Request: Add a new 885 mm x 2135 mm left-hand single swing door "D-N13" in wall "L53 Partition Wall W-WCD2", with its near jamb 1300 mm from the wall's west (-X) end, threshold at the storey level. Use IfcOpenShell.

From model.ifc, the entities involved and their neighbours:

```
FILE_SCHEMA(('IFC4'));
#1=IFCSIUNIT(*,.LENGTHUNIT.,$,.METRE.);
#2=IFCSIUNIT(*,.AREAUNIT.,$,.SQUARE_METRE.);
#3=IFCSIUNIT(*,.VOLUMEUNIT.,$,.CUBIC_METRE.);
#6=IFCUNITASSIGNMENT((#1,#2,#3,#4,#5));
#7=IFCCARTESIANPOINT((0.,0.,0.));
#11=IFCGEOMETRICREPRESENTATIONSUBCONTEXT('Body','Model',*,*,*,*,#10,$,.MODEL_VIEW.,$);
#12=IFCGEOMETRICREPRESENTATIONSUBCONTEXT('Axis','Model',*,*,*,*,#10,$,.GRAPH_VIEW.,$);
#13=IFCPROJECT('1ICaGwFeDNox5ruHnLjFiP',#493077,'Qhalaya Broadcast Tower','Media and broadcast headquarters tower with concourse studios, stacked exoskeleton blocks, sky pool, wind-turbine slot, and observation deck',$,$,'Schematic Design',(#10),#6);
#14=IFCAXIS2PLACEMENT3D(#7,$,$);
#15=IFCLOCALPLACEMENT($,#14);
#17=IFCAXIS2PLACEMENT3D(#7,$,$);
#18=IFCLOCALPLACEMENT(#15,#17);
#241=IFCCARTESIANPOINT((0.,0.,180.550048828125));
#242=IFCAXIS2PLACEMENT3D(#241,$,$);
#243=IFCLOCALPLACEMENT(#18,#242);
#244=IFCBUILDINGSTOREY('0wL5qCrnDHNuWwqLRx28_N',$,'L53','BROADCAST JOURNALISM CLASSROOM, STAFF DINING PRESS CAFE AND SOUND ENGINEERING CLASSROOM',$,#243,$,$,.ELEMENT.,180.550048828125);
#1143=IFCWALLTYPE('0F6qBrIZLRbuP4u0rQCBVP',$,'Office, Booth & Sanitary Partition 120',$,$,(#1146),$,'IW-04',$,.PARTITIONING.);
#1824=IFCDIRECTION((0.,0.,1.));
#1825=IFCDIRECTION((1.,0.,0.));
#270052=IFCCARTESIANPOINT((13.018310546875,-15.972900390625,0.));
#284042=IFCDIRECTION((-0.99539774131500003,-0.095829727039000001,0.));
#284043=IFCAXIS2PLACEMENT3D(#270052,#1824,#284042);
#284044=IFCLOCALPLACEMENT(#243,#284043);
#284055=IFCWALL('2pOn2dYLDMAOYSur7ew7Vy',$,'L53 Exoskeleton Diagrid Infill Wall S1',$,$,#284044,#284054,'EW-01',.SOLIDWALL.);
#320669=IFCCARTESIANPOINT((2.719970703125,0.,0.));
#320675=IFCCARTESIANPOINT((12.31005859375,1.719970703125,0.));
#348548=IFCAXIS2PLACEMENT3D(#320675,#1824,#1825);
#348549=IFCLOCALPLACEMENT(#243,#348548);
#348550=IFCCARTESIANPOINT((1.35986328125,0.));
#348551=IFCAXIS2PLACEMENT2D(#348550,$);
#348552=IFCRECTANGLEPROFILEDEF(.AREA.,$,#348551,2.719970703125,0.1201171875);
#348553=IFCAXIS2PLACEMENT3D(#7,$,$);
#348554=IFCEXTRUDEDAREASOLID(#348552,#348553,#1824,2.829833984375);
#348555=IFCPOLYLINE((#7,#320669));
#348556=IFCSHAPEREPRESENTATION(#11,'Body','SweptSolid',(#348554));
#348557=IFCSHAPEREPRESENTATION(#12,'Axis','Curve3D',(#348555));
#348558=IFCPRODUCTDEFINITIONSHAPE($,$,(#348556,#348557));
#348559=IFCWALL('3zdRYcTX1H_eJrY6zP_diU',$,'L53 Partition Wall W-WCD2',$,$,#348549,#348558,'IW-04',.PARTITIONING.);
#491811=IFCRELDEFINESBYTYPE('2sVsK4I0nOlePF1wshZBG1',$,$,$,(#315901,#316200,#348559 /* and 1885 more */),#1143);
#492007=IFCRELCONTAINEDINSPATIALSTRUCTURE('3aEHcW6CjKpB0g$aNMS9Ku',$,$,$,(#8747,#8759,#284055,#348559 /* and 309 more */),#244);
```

```python
import numpy as np
import ifcopenshell
import ifcopenshell.api.feature
import ifcopenshell.api.geometry
import ifcopenshell.api.root
import ifcopenshell.api.spatial
import ifcopenshell.geom
import ifcopenshell.util.element
import ifcopenshell.util.placement
import ifcopenshell.util.representation
import ifcopenshell.util.shape
import ifcopenshell.util.unit

model = ifcopenshell.open("model.ifc")
unit_scale = ifcopenshell.util.unit.calculate_unit_scale(model)
settings = ifcopenshell.geom.settings()


def volume(element):
    """Net volume in cubic metres, openings subtracted."""
    shape = ifcopenshell.geom.create_shape(settings, element)
    return ifcopenshell.util.shape.get_volume(shape.geometry)


wall = model.by_guid("3zdRYcTX1H_eJrY6zP_diU")
storey = ifcopenshell.util.element.get_container(wall, ifc_class="IfcBuildingStorey")
context = ifcopenshell.util.representation.get_context(model, "Model", "Body", "MODEL_VIEW")
before = volume(wall)

width, height, from_end, sill = 0.885, 2.135, 1.3, 0.0  # metres

# The wall runs along its own X axis, and the end named is its -X end.
wall_shape = ifcopenshell.geom.create_shape(settings, wall)
x, y, z = ifcopenshell.util.shape.get_vertices(wall_shape.geometry).T
start = x.min() + from_end
face, thickness = float(y.min()), float(y.max() - y.min())
wall_matrix = ifcopenshell.util.placement.get_local_placement(wall.ObjectPlacement)
level = ifcopenshell.util.placement.get_local_placement(storey.ObjectPlacement)[2, 3]


def in_wall(x, y):
    """Placement at x, y metres in the wall's axes, at sill height."""
    matrix = wall_matrix.copy()
    matrix[:, 3] = wall_matrix @ np.array([x / unit_scale, y / unit_scale, 0.0, 1.0])
    matrix[2, 3] = level + sill / unit_scale
    return matrix


# Opening: a box that overshoots both wall faces by 50 mm.
opening = ifcopenshell.api.root.create_entity(model, ifc_class="IfcOpeningElement", predefined_type="OPENING")
box = ifcopenshell.api.geometry.add_wall_representation(
    model, context=context, length=width, height=height, thickness=thickness + 0.1
)
ifcopenshell.api.geometry.assign_representation(model, product=opening, representation=box)
ifcopenshell.api.geometry.edit_object_placement(model, product=opening, matrix=in_wall(start, face - 0.05), is_si=False)
ifcopenshell.api.feature.add_feature(model, feature=opening, element=wall)

door = ifcopenshell.api.root.create_entity(model, ifc_class="IfcDoor", name="D-N13", predefined_type="DOOR")
door.OverallWidth, door.OverallHeight = width / unit_scale, height / unit_scale
door.OperationType = "SINGLE_SWING_LEFT"
body = ifcopenshell.api.geometry.add_door_representation(
    model,
    context=context,
    overall_width=door.OverallWidth,
    overall_height=door.OverallHeight,
    operation_type="SINGLE_SWING_LEFT",
    lining_properties={"LiningDepth": thickness / unit_scale, "ThresholdDepth": thickness / unit_scale},
)
ifcopenshell.api.geometry.assign_representation(model, product=door, representation=body)
ifcopenshell.api.spatial.assign_container(model, products=[door], relating_structure=storey)
ifcopenshell.api.feature.add_filling(model, opening=opening, element=door)

# The lining spans the wall, so the door starts at the wall face.
ifcopenshell.api.geometry.edit_object_placement(model, product=door, matrix=in_wall(start, face), is_si=False)

after = volume(wall)

print(f"wall volume {before:.3f} -> {after:.3f} m3")

model.write("model_edited.ifc")
```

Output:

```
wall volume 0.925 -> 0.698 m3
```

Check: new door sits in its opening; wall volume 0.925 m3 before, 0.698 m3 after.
